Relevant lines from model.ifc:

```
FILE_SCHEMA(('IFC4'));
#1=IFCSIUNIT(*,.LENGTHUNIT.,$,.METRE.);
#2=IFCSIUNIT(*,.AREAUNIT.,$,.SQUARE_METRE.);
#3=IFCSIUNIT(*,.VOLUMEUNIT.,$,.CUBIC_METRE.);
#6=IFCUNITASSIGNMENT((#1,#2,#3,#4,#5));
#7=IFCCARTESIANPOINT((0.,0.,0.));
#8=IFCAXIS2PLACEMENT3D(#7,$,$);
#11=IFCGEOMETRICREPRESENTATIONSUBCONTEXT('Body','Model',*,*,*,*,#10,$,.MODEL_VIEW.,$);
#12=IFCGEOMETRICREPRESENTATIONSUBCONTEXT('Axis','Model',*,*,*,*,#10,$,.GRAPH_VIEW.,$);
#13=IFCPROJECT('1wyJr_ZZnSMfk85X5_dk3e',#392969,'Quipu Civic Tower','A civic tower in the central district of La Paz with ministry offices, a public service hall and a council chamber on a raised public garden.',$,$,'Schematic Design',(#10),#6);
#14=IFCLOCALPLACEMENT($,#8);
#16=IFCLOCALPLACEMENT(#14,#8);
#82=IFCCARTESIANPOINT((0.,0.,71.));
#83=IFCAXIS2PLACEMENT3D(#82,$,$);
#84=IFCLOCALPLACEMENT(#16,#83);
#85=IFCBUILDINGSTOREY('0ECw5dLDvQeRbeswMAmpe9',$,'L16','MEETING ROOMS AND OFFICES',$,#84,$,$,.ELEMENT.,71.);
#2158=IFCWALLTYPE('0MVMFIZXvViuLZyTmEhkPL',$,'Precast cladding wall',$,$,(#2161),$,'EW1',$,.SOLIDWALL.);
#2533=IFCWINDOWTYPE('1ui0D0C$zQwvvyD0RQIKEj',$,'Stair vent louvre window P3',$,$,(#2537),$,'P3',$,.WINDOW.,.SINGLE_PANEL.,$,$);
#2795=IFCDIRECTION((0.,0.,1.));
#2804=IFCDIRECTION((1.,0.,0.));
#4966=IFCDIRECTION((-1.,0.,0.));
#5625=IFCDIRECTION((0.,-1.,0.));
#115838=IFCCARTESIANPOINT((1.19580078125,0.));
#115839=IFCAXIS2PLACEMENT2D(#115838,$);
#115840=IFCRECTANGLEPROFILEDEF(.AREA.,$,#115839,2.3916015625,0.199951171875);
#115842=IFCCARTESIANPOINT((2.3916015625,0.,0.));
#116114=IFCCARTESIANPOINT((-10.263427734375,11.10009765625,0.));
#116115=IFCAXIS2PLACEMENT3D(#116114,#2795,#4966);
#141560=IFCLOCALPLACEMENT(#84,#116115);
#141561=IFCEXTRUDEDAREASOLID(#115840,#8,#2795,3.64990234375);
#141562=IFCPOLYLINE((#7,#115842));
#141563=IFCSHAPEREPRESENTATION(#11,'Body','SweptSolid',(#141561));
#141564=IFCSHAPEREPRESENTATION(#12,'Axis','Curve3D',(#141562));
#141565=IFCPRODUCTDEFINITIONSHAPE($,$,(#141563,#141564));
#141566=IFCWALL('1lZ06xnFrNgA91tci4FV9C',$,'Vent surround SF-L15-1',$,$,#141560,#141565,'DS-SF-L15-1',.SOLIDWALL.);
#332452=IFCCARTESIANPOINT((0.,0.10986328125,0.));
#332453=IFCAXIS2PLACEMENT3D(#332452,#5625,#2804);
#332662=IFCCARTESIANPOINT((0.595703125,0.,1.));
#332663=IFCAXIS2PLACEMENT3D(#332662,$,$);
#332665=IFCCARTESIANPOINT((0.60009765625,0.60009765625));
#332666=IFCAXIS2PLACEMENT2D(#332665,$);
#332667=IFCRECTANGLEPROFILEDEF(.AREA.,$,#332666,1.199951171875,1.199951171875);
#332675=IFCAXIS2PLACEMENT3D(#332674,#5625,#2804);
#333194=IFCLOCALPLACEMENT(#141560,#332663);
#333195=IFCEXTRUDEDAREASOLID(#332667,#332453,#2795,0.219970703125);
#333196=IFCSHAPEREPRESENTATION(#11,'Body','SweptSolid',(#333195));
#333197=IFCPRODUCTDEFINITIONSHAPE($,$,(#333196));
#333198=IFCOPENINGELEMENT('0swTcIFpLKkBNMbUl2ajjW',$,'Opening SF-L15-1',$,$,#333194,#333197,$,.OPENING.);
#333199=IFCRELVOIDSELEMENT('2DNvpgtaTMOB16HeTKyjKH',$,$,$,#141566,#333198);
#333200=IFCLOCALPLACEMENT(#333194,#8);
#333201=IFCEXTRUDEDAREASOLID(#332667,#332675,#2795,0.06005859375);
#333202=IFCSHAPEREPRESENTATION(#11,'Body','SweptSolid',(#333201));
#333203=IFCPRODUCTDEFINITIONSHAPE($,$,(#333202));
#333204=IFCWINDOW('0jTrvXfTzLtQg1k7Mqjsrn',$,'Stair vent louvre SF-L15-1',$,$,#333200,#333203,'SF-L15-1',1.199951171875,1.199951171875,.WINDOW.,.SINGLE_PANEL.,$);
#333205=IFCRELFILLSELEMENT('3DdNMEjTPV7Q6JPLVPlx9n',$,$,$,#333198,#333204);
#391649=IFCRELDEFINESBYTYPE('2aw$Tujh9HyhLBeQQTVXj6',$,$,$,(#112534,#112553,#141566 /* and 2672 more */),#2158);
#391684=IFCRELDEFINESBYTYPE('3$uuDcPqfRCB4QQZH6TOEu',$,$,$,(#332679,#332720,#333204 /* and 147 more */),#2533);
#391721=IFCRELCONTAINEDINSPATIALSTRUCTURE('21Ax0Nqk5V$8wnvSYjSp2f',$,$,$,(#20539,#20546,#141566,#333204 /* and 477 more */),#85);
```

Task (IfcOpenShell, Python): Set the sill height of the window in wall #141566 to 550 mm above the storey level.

```python
import numpy as np
import ifcopenshell
import ifcopenshell.api.geometry
import ifcopenshell.geom
import ifcopenshell.util.element
import ifcopenshell.util.placement
import ifcopenshell.util.shape
import ifcopenshell.util.unit

model = ifcopenshell.open("model.ifc")
unit_scale = ifcopenshell.util.unit.calculate_unit_scale(model)

window = model.by_id(333204)
opening = window.FillsVoids[0].RelatingOpeningElement
storey = ifcopenshell.util.element.get_container(window, ifc_class="IfcBuildingStorey")
level = ifcopenshell.util.placement.get_local_placement(storey.ObjectPlacement)[2, 3]

# The opening's origin need not be at the sill, so measure its lowest point.
shape = ifcopenshell.geom.create_shape(ifcopenshell.geom.settings(), opening)
bottom = ifcopenshell.util.shape.get_shape_bottom_elevation(shape, shape.geometry) / unit_scale
dz = level + 0.55 - bottom

shift = np.array([0.0, 0.0, dz])
# The window is placed relative to its opening, so it follows when the opening moves.
matrix = ifcopenshell.util.placement.get_local_placement(opening.ObjectPlacement)
matrix[:3, 3] += shift
ifcopenshell.api.geometry.edit_object_placement(
    model, product=opening, matrix=matrix, is_si=False, should_transform_children=True
)

print(f"moved by {dz * unit_scale:+.3f} m")

model.write("model_rev.ifc")
```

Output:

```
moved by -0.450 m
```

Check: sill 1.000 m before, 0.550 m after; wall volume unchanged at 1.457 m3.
